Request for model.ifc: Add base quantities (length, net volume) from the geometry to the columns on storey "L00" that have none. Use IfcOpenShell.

First a look at what the model holds.

```python
import ifcopenshell
import ifcopenshell.util.element
import ifcopenshell.util.unit

model = ifcopenshell.open("model.ifc")
print(model.schema)
for unit_type in ("LENGTHUNIT", "AREAUNIT", "VOLUMEUNIT"):
    print(unit_type, ifcopenshell.util.unit.calculate_unit_scale(model, unit_type))
storey = next(s for s in model.by_type("IfcBuildingStorey") if s.Name == "L00")
columns = [e for e in ifcopenshell.util.element.get_decomposition(storey) if e.is_a("IfcColumn")]
for e in sorted(columns, key=lambda e: e.id()):
    print(e.id(), e.is_a(), e.Name, list(ifcopenshell.util.element.get_psets(e, qtos_only=True)), sep=" | ")
```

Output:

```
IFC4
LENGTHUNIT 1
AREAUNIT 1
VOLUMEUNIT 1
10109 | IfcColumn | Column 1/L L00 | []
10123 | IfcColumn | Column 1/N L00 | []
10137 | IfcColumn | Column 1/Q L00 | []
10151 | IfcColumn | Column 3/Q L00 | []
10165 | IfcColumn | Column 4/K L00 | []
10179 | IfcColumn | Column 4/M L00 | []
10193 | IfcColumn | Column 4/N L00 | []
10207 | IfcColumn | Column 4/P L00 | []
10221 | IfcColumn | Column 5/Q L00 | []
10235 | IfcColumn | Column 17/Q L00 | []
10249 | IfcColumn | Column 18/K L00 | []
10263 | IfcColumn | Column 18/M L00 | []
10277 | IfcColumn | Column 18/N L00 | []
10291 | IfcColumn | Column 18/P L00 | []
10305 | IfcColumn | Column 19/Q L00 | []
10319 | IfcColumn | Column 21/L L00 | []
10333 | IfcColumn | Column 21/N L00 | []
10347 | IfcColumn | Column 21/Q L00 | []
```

```python
import ifcopenshell
import ifcopenshell.api.pset
import ifcopenshell.geom
import ifcopenshell.util.element
import ifcopenshell.util.shape
import ifcopenshell.util.unit

model = ifcopenshell.open("model.ifc")
unit_scale = ifcopenshell.util.unit.calculate_unit_scale(model)
volume_scale = ifcopenshell.util.unit.calculate_unit_scale(model, "VOLUMEUNIT")
settings = ifcopenshell.geom.settings()

storey = next(s for s in model.by_type("IfcBuildingStorey") if s.Name == "L00")
columns = [e for e in ifcopenshell.util.element.get_decomposition(storey) if e.is_a("IfcColumn")]

for e in sorted(columns, key=lambda e: e.id()):
    if ifcopenshell.util.element.get_psets(e, qtos_only=True, should_inherit=False):
        continue
    # Geometry comes back in metres, in the element's own axes.
    shape = ifcopenshell.geom.create_shape(settings, e)
    values = {
        "Length": ifcopenshell.util.shape.get_z(shape.geometry) / unit_scale,
        "NetVolume": ifcopenshell.util.shape.get_volume(shape.geometry) / volume_scale,
    }
    qto = ifcopenshell.api.pset.add_qto(model, product=e, name="Qto_ColumnBaseQuantities")
    ifcopenshell.api.pset.edit_qto(model, qto=qto, properties=values)
    print(e.id(), {k: round(v, 3) for k, v in values.items()})

model.write("model_edited.ifc")
```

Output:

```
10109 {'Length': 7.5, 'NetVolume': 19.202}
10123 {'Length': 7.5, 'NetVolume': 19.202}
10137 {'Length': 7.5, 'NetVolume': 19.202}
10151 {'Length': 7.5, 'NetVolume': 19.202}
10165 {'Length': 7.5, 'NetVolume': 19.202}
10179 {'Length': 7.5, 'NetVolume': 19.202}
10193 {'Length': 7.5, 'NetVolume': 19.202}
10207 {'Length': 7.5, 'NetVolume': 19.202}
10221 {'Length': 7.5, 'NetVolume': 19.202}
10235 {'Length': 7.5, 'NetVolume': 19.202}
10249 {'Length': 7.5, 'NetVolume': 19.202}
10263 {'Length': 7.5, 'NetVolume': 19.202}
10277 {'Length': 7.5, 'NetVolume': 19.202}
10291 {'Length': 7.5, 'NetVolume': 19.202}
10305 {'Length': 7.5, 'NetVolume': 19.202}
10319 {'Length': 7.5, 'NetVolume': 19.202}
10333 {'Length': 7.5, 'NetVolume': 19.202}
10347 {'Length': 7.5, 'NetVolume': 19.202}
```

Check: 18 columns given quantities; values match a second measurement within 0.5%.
